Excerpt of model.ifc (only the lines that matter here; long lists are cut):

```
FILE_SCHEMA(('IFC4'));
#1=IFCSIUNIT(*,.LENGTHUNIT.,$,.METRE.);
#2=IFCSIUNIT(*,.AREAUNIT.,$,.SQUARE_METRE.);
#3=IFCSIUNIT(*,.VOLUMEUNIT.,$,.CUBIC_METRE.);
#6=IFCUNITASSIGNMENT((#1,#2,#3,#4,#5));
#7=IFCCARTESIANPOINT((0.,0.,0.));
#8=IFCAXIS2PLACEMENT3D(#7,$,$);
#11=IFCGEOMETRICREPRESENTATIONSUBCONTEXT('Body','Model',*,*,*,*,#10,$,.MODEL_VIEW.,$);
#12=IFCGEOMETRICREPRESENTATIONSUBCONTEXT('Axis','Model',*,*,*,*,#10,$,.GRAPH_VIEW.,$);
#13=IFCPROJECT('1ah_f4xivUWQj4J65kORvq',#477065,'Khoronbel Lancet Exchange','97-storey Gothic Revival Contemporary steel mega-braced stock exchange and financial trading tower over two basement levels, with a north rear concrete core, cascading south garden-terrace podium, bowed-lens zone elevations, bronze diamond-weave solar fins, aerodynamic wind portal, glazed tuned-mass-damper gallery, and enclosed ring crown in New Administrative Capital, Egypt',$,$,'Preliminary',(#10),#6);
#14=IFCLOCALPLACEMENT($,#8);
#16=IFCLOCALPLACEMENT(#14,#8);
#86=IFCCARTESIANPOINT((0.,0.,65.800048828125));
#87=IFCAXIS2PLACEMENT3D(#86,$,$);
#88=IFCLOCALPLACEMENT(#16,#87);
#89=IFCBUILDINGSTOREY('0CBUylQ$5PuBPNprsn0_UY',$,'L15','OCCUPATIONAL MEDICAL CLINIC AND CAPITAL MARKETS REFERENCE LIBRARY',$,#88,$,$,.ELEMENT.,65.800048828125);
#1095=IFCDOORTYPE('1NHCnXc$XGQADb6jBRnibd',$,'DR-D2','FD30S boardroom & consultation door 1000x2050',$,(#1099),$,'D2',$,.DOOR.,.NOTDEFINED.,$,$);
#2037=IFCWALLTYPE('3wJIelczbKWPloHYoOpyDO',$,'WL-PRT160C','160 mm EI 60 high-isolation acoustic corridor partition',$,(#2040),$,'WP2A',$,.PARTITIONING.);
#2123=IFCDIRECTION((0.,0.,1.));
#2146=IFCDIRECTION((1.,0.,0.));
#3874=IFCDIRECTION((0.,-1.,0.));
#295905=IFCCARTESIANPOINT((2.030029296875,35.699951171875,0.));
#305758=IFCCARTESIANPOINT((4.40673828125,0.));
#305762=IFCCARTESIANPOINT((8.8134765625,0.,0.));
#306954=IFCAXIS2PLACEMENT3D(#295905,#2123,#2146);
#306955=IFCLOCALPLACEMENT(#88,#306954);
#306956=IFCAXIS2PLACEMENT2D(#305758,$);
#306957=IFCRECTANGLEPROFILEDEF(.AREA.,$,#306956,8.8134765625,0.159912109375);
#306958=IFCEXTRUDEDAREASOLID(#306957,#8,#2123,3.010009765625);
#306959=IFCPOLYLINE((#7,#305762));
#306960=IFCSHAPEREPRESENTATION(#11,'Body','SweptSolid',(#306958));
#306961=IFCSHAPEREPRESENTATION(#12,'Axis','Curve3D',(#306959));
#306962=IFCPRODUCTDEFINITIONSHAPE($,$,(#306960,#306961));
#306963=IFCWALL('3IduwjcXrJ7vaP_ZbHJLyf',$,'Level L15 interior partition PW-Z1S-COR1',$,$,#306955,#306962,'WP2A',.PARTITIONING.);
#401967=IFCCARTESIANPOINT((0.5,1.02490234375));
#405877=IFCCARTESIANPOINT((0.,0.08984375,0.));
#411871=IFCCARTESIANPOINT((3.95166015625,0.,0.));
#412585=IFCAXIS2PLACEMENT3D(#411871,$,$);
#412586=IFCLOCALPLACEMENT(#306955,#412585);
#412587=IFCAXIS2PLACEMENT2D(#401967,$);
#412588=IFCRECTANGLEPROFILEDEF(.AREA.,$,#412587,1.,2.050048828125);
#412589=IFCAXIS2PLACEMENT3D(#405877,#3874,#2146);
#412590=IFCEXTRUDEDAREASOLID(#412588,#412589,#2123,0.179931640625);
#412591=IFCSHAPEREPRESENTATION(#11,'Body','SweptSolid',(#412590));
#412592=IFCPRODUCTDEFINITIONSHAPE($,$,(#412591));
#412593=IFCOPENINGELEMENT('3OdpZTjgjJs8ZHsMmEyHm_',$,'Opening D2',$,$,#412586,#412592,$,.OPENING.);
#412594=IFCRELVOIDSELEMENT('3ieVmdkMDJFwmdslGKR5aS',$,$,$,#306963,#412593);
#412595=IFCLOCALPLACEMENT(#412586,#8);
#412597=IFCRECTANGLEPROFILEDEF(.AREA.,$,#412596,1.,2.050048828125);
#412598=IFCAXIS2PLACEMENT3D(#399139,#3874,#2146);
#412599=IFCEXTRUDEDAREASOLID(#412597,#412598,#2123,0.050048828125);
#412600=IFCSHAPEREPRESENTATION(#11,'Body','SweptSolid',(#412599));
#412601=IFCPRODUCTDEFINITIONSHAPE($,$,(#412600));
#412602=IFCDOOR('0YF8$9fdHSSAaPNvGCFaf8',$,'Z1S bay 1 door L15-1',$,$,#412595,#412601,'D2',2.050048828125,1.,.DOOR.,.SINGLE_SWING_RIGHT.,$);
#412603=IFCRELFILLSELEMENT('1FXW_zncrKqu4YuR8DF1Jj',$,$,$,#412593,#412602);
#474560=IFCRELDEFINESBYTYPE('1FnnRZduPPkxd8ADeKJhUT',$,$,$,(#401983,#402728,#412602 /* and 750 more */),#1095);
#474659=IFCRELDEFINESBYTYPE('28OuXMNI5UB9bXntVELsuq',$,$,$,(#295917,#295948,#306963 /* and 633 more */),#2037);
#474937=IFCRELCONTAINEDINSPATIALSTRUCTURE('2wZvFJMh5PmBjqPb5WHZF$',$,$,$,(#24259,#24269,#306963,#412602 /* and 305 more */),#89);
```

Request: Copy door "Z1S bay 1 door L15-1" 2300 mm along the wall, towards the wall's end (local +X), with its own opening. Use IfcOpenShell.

```python
import ifcopenshell
import ifcopenshell.api.feature
import ifcopenshell.api.geometry
import ifcopenshell.api.root
import ifcopenshell.geom
import ifcopenshell.util.element
import ifcopenshell.util.placement
import ifcopenshell.util.shape

model = ifcopenshell.open("model.ifc")
settings = ifcopenshell.geom.settings()


def volume(element):
    """Net volume in cubic metres, openings subtracted."""
    shape = ifcopenshell.geom.create_shape(settings, element)
    return ifcopenshell.util.shape.get_volume(shape.geometry)


door = model.by_id(412602)
opening = door.FillsVoids[0].RelatingOpeningElement
wall = opening.VoidsElements[0].RelatingBuildingElement
before = volume(wall)
shift = ifcopenshell.util.placement.get_local_placement(wall.ObjectPlacement)[:3, 0] * 2.3

# copy_class copies the void relationship, type, container and properties, but no geometry.
new_opening = ifcopenshell.api.root.copy_class(model, product=opening)
new_opening.Representation = ifcopenshell.util.element.copy_deep(
    model, opening.Representation, exclude=["IfcGeometricRepresentationContext", "IfcRepresentationMap"]
)
new_door = ifcopenshell.api.root.copy_class(model, product=door)
new_door.Representation = ifcopenshell.util.element.copy_deep(
    model, door.Representation, exclude=["IfcGeometricRepresentationContext", "IfcRepresentationMap"]
)
new_door.Tag = None
ifcopenshell.api.feature.add_filling(model, opening=new_opening, element=new_door)

for old, new in ((opening, new_opening), (door, new_door)):
    matrix = ifcopenshell.util.placement.get_local_placement(old.ObjectPlacement)
    matrix[:3, 3] += shift
    ifcopenshell.api.geometry.edit_object_placement(model, product=new, matrix=matrix, is_si=False)

after = volume(wall)

print(f"wall volume {before:.3f} -> {after:.3f} m3")

model.write("model_v2.ifc")
```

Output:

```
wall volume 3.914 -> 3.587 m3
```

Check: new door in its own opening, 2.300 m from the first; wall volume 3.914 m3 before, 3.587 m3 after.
